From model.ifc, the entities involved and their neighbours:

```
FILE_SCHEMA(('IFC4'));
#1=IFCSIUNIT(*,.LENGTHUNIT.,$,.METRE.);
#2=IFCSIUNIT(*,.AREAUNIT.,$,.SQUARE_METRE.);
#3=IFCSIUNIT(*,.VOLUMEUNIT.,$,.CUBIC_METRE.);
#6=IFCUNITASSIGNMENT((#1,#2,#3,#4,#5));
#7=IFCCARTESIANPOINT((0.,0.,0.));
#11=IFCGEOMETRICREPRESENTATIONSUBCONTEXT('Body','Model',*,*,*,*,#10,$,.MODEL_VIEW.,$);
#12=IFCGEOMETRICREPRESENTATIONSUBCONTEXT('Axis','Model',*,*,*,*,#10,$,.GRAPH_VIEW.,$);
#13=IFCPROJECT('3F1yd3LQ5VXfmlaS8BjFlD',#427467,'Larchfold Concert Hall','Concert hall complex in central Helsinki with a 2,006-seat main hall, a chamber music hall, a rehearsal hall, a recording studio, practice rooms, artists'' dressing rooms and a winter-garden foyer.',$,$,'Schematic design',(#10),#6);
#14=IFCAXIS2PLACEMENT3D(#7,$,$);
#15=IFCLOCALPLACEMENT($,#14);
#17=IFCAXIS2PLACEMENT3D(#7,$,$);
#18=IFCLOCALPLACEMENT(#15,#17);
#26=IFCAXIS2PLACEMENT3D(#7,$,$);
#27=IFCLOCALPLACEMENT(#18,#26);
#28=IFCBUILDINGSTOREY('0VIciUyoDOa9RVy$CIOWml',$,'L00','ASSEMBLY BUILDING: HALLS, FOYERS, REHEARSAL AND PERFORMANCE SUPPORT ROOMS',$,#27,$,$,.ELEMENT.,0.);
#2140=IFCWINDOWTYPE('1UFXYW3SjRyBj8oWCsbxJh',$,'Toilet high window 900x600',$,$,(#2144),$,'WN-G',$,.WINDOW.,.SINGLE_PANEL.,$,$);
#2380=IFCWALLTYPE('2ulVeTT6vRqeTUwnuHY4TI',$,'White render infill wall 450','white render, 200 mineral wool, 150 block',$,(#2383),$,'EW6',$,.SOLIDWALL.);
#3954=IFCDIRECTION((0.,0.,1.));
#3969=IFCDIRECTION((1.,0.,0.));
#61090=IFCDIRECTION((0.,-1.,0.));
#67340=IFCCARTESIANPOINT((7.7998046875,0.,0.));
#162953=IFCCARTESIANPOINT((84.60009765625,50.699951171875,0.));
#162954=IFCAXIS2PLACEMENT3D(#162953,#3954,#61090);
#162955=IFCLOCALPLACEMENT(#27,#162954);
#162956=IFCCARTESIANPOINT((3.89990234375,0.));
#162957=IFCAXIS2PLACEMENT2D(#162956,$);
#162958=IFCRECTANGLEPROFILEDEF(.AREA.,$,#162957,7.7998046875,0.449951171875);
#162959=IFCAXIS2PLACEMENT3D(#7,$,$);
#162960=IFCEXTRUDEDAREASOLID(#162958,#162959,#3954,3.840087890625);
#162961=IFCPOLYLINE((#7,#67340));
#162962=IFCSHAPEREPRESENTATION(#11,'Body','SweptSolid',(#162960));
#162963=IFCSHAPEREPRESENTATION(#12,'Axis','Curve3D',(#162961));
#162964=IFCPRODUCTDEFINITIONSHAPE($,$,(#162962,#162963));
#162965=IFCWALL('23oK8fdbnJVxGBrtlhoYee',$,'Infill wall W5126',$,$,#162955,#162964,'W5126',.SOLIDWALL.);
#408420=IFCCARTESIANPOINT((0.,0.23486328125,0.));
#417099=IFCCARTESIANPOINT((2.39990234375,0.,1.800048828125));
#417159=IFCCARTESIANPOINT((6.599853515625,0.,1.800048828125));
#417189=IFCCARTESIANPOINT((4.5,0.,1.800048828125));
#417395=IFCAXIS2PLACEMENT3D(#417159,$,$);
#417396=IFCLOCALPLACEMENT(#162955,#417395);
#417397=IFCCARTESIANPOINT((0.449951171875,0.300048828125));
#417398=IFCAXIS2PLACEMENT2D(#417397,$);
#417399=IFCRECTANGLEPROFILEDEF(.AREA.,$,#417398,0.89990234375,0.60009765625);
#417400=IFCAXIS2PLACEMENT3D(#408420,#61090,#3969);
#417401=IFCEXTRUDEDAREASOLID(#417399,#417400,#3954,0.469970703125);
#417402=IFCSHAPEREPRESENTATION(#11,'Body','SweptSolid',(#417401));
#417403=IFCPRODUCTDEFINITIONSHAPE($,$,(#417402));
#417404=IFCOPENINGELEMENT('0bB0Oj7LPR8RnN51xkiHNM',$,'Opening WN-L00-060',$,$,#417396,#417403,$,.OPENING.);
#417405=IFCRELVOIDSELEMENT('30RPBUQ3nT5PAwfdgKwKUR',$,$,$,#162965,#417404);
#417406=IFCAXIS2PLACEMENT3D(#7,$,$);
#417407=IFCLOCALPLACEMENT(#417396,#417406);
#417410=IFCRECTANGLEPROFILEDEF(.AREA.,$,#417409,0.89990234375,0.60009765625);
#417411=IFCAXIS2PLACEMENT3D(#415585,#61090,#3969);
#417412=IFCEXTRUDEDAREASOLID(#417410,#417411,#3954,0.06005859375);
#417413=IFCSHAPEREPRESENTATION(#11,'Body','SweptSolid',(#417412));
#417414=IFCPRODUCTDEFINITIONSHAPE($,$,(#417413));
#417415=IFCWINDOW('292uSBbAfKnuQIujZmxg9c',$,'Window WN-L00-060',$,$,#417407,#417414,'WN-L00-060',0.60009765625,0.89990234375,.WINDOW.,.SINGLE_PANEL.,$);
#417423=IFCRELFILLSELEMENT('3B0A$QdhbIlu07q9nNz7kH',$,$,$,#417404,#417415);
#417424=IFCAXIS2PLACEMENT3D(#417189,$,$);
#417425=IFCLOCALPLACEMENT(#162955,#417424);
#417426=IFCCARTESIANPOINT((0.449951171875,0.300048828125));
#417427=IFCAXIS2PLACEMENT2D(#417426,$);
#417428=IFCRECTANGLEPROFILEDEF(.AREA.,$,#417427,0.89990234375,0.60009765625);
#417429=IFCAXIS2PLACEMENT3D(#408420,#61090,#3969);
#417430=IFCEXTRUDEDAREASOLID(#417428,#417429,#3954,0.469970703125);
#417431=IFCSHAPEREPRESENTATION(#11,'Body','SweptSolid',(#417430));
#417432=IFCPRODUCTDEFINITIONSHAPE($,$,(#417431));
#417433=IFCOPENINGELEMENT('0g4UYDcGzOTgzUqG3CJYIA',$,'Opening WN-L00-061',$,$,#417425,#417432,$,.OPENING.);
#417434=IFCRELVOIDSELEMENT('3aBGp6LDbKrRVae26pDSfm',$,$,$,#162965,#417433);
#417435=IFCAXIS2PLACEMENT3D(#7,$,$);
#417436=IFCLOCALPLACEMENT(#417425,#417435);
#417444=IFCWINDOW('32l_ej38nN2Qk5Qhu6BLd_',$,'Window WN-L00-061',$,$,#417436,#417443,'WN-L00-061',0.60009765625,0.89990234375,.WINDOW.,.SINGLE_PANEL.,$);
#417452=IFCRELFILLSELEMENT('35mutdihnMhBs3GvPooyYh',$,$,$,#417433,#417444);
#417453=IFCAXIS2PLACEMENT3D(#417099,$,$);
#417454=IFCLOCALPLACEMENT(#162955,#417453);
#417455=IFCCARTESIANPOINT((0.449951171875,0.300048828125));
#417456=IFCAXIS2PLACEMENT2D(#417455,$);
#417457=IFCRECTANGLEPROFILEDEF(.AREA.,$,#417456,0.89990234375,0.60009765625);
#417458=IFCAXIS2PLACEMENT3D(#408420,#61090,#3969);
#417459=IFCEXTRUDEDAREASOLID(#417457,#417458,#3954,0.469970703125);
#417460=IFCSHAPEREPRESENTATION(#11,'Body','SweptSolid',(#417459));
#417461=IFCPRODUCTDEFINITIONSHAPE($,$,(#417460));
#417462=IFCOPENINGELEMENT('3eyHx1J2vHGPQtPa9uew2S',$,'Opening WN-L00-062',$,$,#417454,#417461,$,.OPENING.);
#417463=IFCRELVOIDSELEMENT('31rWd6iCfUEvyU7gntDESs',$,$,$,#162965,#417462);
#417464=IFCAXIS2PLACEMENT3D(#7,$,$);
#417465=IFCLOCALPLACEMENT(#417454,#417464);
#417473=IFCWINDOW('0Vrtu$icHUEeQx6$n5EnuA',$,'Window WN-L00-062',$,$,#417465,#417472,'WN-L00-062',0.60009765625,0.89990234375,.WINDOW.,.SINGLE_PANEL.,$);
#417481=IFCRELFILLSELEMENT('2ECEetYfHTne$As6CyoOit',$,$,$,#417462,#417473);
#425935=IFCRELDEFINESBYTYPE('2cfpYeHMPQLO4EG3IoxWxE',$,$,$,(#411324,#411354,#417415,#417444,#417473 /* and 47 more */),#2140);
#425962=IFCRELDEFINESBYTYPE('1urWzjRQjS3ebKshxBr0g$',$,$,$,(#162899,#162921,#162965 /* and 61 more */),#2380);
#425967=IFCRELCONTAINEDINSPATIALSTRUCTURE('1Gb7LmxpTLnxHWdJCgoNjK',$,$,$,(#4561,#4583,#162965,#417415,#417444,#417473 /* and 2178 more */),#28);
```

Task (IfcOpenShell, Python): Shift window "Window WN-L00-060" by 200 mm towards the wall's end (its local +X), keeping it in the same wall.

```python
import ifcopenshell
import ifcopenshell.api.geometry
import ifcopenshell.util.placement
import ifcopenshell.util.unit

model = ifcopenshell.open("model.ifc")
unit_scale = ifcopenshell.util.unit.calculate_unit_scale(model)

window = model.by_guid("292uSBbAfKnuQIujZmxg9c")
opening = window.FillsVoids[0].RelatingOpeningElement
wall = opening.VoidsElements[0].RelatingBuildingElement

wall_matrix = ifcopenshell.util.placement.get_local_placement(wall.ObjectPlacement)
shift = wall_matrix[:3, 0] * 0.2 / unit_scale
before = ifcopenshell.util.placement.get_local_placement(window.ObjectPlacement)[:3, 3].copy()

# The window is placed relative to its opening, so it follows when the opening moves.
matrix = ifcopenshell.util.placement.get_local_placement(opening.ObjectPlacement)
matrix[:3, 3] += shift
ifcopenshell.api.geometry.edit_object_placement(
    model, product=opening, matrix=matrix, is_si=False, should_transform_children=True
)

after = ifcopenshell.util.placement.get_local_placement(window.ObjectPlacement)[:3, 3]
print("window moved by", (after - before).round(3) + 0.0)

model.write("model_rev.ifc")
```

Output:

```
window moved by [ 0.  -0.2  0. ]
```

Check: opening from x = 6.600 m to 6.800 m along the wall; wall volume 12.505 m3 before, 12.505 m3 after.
